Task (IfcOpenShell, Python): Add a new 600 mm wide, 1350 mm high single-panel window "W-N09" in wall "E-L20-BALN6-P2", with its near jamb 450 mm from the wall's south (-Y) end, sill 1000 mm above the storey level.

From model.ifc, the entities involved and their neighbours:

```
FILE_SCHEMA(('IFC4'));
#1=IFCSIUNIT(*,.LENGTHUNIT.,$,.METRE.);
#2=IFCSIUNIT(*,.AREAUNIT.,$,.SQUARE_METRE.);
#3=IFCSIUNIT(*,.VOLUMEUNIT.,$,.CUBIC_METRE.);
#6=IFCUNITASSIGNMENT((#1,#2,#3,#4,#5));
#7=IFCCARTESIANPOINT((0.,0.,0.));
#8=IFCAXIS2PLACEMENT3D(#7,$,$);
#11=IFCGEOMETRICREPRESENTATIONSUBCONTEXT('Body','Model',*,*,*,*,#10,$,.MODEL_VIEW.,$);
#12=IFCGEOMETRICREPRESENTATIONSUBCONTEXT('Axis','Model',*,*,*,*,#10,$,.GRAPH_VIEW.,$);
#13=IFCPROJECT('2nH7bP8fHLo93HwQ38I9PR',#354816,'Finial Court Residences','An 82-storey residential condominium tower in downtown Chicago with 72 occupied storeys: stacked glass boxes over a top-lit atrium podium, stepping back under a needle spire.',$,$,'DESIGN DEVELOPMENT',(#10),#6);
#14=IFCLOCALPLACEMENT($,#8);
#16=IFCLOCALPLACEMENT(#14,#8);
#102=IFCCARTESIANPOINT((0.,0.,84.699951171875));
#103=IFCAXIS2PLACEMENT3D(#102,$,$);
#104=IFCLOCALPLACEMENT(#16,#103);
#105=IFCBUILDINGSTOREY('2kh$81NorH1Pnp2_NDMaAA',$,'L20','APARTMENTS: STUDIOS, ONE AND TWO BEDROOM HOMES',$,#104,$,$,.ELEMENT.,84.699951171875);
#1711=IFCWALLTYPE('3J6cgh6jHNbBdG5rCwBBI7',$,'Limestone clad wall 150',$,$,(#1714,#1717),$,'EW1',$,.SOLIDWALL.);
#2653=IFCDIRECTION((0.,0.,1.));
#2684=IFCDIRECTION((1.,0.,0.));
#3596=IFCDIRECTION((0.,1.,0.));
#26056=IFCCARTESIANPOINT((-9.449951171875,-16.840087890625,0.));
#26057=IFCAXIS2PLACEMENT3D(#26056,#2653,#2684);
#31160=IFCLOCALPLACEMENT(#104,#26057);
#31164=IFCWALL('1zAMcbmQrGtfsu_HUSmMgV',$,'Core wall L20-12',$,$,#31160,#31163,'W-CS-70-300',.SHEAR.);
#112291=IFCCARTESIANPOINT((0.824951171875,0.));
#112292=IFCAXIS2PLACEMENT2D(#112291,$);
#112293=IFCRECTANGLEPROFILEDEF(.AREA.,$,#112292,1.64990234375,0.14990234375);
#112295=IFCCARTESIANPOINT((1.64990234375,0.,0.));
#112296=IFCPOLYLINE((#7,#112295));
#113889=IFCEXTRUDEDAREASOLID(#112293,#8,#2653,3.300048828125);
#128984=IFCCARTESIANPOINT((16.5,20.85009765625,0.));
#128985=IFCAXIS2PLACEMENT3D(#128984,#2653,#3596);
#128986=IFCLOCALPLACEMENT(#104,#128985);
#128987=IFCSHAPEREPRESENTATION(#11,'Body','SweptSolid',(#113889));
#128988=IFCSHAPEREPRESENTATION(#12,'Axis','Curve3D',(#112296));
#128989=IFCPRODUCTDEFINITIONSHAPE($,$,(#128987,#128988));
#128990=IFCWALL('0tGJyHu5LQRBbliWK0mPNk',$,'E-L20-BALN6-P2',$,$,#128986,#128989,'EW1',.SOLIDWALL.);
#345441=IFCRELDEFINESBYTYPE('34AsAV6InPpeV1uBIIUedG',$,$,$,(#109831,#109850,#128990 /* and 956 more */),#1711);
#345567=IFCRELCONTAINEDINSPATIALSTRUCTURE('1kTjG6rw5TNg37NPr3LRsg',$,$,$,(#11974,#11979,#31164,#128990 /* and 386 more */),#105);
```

```python
import numpy as np
import ifcopenshell
import ifcopenshell.api.feature
import ifcopenshell.api.geometry
import ifcopenshell.api.root
import ifcopenshell.api.spatial
import ifcopenshell.geom
import ifcopenshell.util.element
import ifcopenshell.util.placement
import ifcopenshell.util.representation
import ifcopenshell.util.shape
import ifcopenshell.util.unit

model = ifcopenshell.open("model.ifc")
unit_scale = ifcopenshell.util.unit.calculate_unit_scale(model)
settings = ifcopenshell.geom.settings()


def volume(element):
    """Net volume in cubic metres, openings subtracted."""
    shape = ifcopenshell.geom.create_shape(settings, element)
    return ifcopenshell.util.shape.get_volume(shape.geometry)


wall = model.by_guid("0tGJyHu5LQRBbliWK0mPNk")
storey = ifcopenshell.util.element.get_container(wall, ifc_class="IfcBuildingStorey")
context = ifcopenshell.util.representation.get_context(model, "Model", "Body", "MODEL_VIEW")
before = volume(wall)

width, height, from_end, sill = 0.6, 1.35, 0.45, 1  # metres

# The wall runs along its own X axis, and the end named is its -X end.
wall_shape = ifcopenshell.geom.create_shape(settings, wall)
x, y, z = ifcopenshell.util.shape.get_vertices(wall_shape.geometry).T
start = x.min() + from_end
face, thickness = float(y.min()), float(y.max() - y.min())
wall_matrix = ifcopenshell.util.placement.get_local_placement(wall.ObjectPlacement)
level = ifcopenshell.util.placement.get_local_placement(storey.ObjectPlacement)[2, 3]


def in_wall(x, y):
    """Placement at x, y metres in the wall's axes, at sill height."""
    matrix = wall_matrix.copy()
    matrix[:, 3] = wall_matrix @ np.array([x / unit_scale, y / unit_scale, 0.0, 1.0])
    matrix[2, 3] = level + sill / unit_scale
    return matrix


# Opening: a box that overshoots both wall faces by 50 mm.
opening = ifcopenshell.api.root.create_entity(model, ifc_class="IfcOpeningElement", predefined_type="OPENING")
box = ifcopenshell.api.geometry.add_wall_representation(
    model, context=context, length=width, height=height, thickness=thickness + 0.1
)
ifcopenshell.api.geometry.assign_representation(model, product=opening, representation=box)
ifcopenshell.api.geometry.edit_object_placement(model, product=opening, matrix=in_wall(start, face - 0.05), is_si=False)
ifcopenshell.api.feature.add_feature(model, feature=opening, element=wall)

window = ifcopenshell.api.root.create_entity(model, ifc_class="IfcWindow", name="W-N09", predefined_type="WINDOW")
window.OverallWidth, window.OverallHeight = width / unit_scale, height / unit_scale
window.PartitioningType = "SINGLE_PANEL"
body = ifcopenshell.api.geometry.add_window_representation(
    model,
    context=context,
    overall_width=window.OverallWidth,
    overall_height=window.OverallHeight,
    partition_type="SINGLE_PANEL",
)
ifcopenshell.api.geometry.assign_representation(model, product=window, representation=body)
ifcopenshell.api.spatial.assign_container(model, products=[window], relating_structure=storey)
ifcopenshell.api.feature.add_filling(model, opening=opening, element=window)

# Centre the window in the wall's thickness.
ifcopenshell.api.geometry.edit_object_placement(model, product=window, matrix=in_wall(start, face), is_si=False)
window_shape = ifcopenshell.geom.create_shape(settings, window)
depth = ifcopenshell.util.shape.get_vertices(window_shape.geometry)[:, 1]
offset = face + thickness / 2 - (depth.min() + depth.max()) / 2
ifcopenshell.api.geometry.edit_object_placement(model, product=window, matrix=in_wall(start, offset), is_si=False)

after = volume(wall)

print(f"wall volume {before:.3f} -> {after:.3f} m3")

model.write("model_v2.ifc")
```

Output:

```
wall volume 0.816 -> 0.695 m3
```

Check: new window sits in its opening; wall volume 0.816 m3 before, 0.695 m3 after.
